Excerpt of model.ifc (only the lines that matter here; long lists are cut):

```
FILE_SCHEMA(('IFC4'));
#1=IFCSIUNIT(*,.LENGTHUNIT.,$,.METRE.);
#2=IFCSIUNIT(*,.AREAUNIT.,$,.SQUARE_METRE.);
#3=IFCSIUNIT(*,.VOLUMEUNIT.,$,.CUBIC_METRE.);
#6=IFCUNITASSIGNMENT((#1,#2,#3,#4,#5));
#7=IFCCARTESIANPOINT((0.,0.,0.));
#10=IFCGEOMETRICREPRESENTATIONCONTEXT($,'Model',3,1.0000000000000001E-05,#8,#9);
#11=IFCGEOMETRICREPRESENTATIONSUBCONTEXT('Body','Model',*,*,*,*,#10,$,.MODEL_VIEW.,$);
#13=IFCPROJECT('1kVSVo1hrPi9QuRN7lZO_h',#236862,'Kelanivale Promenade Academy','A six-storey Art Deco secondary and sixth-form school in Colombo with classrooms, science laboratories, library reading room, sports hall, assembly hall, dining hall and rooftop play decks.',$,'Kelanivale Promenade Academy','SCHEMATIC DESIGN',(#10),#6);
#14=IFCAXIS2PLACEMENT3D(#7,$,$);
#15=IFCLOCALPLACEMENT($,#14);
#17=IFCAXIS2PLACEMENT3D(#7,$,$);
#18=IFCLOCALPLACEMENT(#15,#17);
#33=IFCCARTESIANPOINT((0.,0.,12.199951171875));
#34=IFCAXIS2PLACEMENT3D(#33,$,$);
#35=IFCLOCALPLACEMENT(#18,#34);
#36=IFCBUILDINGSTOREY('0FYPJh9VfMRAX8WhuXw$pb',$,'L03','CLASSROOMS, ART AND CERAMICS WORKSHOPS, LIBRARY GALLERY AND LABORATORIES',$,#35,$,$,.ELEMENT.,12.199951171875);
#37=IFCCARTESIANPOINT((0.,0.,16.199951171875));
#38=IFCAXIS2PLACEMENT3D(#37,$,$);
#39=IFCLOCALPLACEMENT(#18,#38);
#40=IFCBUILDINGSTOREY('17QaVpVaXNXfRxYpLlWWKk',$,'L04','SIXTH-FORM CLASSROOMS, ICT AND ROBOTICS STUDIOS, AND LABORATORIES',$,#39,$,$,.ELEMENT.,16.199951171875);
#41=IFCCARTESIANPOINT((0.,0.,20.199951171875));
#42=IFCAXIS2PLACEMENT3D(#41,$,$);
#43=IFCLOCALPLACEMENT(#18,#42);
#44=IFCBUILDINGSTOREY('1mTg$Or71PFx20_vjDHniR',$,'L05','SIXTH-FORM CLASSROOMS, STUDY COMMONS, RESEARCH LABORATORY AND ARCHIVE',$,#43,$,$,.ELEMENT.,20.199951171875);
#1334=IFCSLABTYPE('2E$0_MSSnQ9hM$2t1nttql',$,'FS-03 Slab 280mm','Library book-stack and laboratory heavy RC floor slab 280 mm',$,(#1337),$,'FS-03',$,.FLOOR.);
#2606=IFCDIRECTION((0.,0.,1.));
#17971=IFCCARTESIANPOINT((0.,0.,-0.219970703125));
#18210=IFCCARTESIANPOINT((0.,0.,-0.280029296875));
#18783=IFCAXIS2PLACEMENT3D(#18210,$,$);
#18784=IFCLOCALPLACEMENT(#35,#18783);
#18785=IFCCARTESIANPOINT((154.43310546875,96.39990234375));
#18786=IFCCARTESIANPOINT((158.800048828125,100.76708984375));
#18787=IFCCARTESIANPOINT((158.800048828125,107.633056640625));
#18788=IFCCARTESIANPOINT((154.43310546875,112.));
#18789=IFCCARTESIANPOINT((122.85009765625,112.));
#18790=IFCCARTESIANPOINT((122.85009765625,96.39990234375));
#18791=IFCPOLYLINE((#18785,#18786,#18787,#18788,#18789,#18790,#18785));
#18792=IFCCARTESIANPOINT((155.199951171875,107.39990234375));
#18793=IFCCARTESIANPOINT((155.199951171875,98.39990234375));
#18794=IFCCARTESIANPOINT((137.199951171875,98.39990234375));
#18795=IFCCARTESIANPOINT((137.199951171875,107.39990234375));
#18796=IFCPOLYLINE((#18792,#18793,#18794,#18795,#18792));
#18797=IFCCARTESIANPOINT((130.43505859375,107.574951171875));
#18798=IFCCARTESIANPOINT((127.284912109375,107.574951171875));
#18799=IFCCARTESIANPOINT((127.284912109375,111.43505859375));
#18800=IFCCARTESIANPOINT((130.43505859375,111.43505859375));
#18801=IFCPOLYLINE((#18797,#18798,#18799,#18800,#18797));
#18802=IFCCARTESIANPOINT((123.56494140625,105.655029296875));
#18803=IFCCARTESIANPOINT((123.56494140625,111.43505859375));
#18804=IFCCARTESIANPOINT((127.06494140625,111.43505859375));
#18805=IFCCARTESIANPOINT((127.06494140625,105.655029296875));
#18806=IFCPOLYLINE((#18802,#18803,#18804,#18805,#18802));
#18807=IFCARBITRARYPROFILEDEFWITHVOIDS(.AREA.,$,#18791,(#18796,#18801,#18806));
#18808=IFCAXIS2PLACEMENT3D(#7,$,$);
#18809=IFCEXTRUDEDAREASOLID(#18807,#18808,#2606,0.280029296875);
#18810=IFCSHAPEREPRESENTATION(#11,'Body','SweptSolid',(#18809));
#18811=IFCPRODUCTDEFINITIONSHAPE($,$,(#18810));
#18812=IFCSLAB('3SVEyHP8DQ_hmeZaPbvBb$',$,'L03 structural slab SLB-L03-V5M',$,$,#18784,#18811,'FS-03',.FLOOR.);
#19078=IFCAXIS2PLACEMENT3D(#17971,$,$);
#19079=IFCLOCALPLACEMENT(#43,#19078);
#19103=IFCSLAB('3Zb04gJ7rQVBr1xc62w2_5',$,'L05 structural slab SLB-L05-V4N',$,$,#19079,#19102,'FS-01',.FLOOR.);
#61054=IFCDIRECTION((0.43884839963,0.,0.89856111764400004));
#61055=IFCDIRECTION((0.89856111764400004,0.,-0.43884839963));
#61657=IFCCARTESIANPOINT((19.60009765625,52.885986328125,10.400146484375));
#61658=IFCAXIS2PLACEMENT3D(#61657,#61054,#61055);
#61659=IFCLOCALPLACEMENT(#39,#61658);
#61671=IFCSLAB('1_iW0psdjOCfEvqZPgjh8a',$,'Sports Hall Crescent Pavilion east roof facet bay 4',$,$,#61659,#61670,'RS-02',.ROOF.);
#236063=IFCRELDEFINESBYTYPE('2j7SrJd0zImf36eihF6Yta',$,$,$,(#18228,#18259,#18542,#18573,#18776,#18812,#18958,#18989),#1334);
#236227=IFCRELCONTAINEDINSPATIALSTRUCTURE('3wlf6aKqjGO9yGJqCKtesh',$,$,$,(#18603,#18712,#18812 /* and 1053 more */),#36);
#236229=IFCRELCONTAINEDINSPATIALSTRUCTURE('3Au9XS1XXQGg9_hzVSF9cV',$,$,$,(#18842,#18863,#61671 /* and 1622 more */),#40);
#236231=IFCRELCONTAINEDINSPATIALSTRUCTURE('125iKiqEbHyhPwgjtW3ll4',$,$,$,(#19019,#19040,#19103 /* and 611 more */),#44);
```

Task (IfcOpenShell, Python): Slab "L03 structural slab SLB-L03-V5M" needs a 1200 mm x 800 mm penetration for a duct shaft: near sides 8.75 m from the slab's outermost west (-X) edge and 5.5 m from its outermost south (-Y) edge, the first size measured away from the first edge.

```python
import numpy as np
import ifcopenshell
import ifcopenshell.api.feature
import ifcopenshell.api.geometry
import ifcopenshell.api.root
import ifcopenshell.geom
import ifcopenshell.util.placement
import ifcopenshell.util.representation
import ifcopenshell.util.shape
import ifcopenshell.util.unit

model = ifcopenshell.open("model.ifc")
unit_scale = ifcopenshell.util.unit.calculate_unit_scale(model)
settings = ifcopenshell.geom.settings()


def volume(element):
    """Net volume in cubic metres, openings subtracted."""
    shape = ifcopenshell.geom.create_shape(settings, element)
    return ifcopenshell.util.shape.get_volume(shape.geometry)


slab = model.by_id(18812)
before = volume(slab)

# Extent in the slab's own axes, in metres. The edges named are its -X and -Y sides.
slab_shape = ifcopenshell.geom.create_shape(settings, slab)
vertices = ifcopenshell.util.shape.get_vertices(slab_shape.geometry)
x_min, y_min, bottom = vertices.min(axis=0)
top = vertices[:, 2].max()

opening = ifcopenshell.api.root.create_entity(model, ifc_class="IfcOpeningElement", name="Duct shaft opening", predefined_type="OPENING")
context = ifcopenshell.util.representation.get_context(model, "Model", "Body", "MODEL_VIEW")
width, depth = 1.2, 0.8
outline = [(0.0, 0.0), (width, 0.0), (width, depth), (0.0, depth), (0.0, 0.0)]
# Overshoot both faces by 50 mm so the cut is clean.
shape = ifcopenshell.api.geometry.add_slab_representation(
    model, context=context, depth=top - bottom + 0.1, polyline=outline
)
ifcopenshell.api.geometry.assign_representation(model, product=opening, representation=shape)

matrix = ifcopenshell.util.placement.get_local_placement(slab.ObjectPlacement)
matrix[:, 3] = matrix @ np.append(np.array([x_min + 8.75, y_min + 5.5, bottom - 0.05]) / unit_scale, 1.0)
ifcopenshell.api.geometry.edit_object_placement(model, product=opening, matrix=matrix, is_si=False)
ifcopenshell.api.feature.add_feature(model, feature=opening, element=slab)

after = volume(slab)

print(f"slab volume {before:.3f} -> {after:.3f} m3")

model.write("model_edited.ifc")
```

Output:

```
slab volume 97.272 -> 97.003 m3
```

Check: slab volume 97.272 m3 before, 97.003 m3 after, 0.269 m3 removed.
